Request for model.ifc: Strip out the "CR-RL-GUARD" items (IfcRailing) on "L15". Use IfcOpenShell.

First a look at what the model holds.

```python
import ifcopenshell
import ifcopenshell.util.element

model = ifcopenshell.open("model.ifc")
print(model.schema)
storey = next(s for s in model.by_type("IfcBuildingStorey") if s.Name == "L15")
railings = [e for e in ifcopenshell.util.element.get_decomposition(storey) if e.is_a("IfcRailing")]
seen = {}
for e in railings:
    element_type = ifcopenshell.util.element.get_type(e)
    name = element_type.Name if element_type not in (None, e) else None
    seen[name] = seen.get(name, 0) + 1
for name, count in sorted(seen.items(), key=str):
    print(count, "x", name)
```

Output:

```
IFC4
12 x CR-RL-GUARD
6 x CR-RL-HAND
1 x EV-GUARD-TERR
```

```python
import ifcopenshell
import ifcopenshell.api.root
import ifcopenshell.util.element

model = ifcopenshell.open("model.ifc")

storey = next(s for s in model.by_type("IfcBuildingStorey") if s.Name == "L15")
railings = [e for e in ifcopenshell.util.element.get_decomposition(storey) if e.is_a("IfcRailing")]
targets = [e for e in railings if (t := ifcopenshell.util.element.get_type(e)) not in (None, e) and t.Name == "CR-RL-GUARD"]

for e in targets:
    ifcopenshell.api.root.remove_product(model, product=e)
print(len(targets), "removed")

model.write("model-out.ifc")
```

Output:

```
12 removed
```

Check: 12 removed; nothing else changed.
